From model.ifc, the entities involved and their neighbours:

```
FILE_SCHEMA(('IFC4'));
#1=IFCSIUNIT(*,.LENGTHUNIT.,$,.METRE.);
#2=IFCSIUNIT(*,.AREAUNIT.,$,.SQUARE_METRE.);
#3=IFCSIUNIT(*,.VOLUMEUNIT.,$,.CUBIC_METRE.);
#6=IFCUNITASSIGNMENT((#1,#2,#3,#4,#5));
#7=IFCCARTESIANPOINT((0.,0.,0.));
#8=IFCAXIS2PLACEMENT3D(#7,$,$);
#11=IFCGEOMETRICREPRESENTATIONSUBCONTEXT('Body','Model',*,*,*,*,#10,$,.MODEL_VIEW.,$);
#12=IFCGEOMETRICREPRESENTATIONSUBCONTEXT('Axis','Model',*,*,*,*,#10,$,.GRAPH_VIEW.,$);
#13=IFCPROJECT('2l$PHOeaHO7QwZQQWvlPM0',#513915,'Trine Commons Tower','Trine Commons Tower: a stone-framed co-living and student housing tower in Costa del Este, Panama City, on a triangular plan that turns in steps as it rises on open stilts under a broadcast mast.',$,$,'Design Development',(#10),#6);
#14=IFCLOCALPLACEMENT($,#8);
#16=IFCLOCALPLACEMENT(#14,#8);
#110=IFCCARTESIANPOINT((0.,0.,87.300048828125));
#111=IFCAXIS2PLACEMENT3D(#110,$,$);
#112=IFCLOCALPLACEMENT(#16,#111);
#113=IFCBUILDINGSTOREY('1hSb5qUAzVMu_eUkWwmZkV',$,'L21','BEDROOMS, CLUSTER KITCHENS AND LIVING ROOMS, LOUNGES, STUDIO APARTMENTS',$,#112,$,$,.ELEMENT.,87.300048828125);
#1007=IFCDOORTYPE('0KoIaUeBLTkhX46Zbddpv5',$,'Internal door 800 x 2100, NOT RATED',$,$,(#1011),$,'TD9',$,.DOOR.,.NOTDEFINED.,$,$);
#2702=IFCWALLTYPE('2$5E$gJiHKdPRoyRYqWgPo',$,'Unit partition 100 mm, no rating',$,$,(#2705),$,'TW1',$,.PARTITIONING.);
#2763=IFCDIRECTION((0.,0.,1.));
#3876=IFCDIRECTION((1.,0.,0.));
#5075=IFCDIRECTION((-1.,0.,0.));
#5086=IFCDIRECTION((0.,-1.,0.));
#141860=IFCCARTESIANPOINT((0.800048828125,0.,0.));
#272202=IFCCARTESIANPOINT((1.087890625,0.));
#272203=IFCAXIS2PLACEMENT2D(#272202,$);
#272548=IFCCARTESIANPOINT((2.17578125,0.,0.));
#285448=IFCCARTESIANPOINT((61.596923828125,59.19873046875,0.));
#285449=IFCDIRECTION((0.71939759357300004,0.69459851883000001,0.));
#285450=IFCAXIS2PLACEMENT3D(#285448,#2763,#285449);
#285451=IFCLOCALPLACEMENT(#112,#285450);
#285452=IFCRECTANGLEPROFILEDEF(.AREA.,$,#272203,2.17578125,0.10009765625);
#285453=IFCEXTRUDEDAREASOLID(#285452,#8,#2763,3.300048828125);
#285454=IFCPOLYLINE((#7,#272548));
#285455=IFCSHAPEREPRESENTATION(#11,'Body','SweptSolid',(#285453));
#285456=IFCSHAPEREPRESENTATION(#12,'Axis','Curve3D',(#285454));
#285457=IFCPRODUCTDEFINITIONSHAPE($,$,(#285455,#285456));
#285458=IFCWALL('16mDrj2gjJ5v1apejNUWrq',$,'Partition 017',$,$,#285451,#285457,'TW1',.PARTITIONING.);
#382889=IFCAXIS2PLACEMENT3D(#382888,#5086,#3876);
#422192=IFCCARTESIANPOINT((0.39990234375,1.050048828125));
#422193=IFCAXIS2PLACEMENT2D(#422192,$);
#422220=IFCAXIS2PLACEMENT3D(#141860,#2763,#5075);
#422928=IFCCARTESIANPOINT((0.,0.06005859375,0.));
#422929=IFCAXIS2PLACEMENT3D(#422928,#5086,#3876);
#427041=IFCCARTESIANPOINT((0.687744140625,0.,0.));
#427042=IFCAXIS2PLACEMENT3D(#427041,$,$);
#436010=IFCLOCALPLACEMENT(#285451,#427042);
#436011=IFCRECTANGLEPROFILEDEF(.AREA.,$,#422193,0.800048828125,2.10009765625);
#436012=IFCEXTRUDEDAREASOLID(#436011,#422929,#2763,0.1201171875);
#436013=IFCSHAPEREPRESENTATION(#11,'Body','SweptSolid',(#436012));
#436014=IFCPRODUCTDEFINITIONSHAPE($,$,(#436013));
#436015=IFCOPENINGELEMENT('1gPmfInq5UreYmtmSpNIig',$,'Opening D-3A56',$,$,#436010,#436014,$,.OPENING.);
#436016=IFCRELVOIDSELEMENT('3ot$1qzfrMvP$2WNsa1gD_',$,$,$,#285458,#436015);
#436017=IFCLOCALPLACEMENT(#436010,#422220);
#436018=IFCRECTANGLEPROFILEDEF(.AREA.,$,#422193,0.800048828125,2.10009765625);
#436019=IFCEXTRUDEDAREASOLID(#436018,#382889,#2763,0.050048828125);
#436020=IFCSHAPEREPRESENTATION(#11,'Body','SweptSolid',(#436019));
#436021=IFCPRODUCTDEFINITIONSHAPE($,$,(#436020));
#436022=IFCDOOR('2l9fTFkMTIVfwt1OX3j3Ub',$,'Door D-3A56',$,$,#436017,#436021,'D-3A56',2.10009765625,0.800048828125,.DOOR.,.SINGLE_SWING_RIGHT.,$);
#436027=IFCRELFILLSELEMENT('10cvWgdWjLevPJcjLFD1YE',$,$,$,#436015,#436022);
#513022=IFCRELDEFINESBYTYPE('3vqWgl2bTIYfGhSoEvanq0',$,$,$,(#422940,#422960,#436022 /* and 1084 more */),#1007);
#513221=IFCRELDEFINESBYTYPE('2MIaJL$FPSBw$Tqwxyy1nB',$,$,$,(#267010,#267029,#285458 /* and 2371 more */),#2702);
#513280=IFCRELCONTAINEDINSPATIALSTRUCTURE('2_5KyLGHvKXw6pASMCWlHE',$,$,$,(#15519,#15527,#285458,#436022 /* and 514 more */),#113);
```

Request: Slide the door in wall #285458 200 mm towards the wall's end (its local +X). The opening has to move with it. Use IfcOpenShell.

```python
import ifcopenshell
import ifcopenshell.api.geometry
import ifcopenshell.util.placement
import ifcopenshell.util.unit

model = ifcopenshell.open("model.ifc")
unit_scale = ifcopenshell.util.unit.calculate_unit_scale(model)

door = model.by_id(436022)
opening = door.FillsVoids[0].RelatingOpeningElement
wall = opening.VoidsElements[0].RelatingBuildingElement

wall_matrix = ifcopenshell.util.placement.get_local_placement(wall.ObjectPlacement)
shift = wall_matrix[:3, 0] * 0.2 / unit_scale
before = ifcopenshell.util.placement.get_local_placement(door.ObjectPlacement)[:3, 3].copy()

# The door is placed relative to its opening, so it follows when the opening moves.
matrix = ifcopenshell.util.placement.get_local_placement(opening.ObjectPlacement)
matrix[:3, 3] += shift
ifcopenshell.api.geometry.edit_object_placement(
    model, product=opening, matrix=matrix, is_si=False, should_transform_children=True
)

after = ifcopenshell.util.placement.get_local_placement(door.ObjectPlacement)[:3, 3]
print("door moved by", (after - before).round(3) + 0.0)

model.write("model_updated.ifc")
```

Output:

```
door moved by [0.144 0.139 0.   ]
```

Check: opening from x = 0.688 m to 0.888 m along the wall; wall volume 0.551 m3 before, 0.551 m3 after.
